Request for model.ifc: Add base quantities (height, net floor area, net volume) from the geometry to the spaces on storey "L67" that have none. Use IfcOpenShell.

First a look at what the model holds.

```python
import ifcopenshell
import ifcopenshell.util.element
import ifcopenshell.util.unit

model = ifcopenshell.open("model.ifc")
print(model.schema)
for unit_type in ("LENGTHUNIT", "AREAUNIT", "VOLUMEUNIT"):
    print(unit_type, ifcopenshell.util.unit.calculate_unit_scale(model, unit_type))
storey = next(s for s in model.by_type("IfcBuildingStorey") if s.Name == "L67")
spaces = [e for e in ifcopenshell.util.element.get_decomposition(storey) if e.is_a("IfcSpace")]
for e in sorted(spaces, key=lambda e: e.id()):
    print(e.id(), e.is_a(), e.Name, list(ifcopenshell.util.element.get_psets(e, qtos_only=True)), sep=" | ")
```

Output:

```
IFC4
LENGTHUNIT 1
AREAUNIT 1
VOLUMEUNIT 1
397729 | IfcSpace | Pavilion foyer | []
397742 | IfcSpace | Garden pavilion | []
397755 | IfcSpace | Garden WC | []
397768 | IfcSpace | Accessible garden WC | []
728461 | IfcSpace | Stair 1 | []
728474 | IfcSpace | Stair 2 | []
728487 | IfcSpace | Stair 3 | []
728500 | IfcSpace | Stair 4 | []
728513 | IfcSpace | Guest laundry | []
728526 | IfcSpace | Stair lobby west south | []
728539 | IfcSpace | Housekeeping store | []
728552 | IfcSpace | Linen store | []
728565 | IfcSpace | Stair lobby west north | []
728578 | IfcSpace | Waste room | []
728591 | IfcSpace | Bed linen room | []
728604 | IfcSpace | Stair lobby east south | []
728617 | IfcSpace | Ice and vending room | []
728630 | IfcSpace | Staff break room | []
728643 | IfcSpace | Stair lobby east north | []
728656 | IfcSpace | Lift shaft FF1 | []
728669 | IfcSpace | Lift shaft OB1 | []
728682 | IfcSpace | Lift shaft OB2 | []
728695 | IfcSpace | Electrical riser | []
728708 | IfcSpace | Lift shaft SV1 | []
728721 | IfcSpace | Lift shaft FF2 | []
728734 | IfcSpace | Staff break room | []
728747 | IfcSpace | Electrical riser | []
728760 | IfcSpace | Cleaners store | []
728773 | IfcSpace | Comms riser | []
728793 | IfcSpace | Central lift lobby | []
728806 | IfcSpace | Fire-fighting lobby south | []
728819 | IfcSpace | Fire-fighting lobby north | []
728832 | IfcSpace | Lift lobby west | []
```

```python
import ifcopenshell
import ifcopenshell.api.pset
import ifcopenshell.geom
import ifcopenshell.util.element
import ifcopenshell.util.shape
import ifcopenshell.util.unit

model = ifcopenshell.open("model.ifc")
unit_scale = ifcopenshell.util.unit.calculate_unit_scale(model)
area_scale = ifcopenshell.util.unit.calculate_unit_scale(model, "AREAUNIT")
volume_scale = ifcopenshell.util.unit.calculate_unit_scale(model, "VOLUMEUNIT")
settings = ifcopenshell.geom.settings()

storey = next(s for s in model.by_type("IfcBuildingStorey") if s.Name == "L67")
spaces = [e for e in ifcopenshell.util.element.get_decomposition(storey) if e.is_a("IfcSpace")]

for e in sorted(spaces, key=lambda e: e.id()):
    if ifcopenshell.util.element.get_psets(e, qtos_only=True, should_inherit=False):
        continue
    # Geometry comes back in metres, in the element's own axes.
    shape = ifcopenshell.geom.create_shape(settings, e)
    values = {
        "Height": ifcopenshell.util.shape.get_z(shape.geometry) / unit_scale,
        "NetFloorArea": ifcopenshell.util.shape.get_footprint_area(shape.geometry) / area_scale,
        "NetVolume": ifcopenshell.util.shape.get_volume(shape.geometry) / volume_scale,
    }
    qto = ifcopenshell.api.pset.add_qto(model, product=e, name="Qto_SpaceBaseQuantities")
    ifcopenshell.api.pset.edit_qto(model, qto=qto, properties=values)
    print(e.id(), {k: round(v, 3) for k, v in values.items()})

model.write("model_edited.ifc")
```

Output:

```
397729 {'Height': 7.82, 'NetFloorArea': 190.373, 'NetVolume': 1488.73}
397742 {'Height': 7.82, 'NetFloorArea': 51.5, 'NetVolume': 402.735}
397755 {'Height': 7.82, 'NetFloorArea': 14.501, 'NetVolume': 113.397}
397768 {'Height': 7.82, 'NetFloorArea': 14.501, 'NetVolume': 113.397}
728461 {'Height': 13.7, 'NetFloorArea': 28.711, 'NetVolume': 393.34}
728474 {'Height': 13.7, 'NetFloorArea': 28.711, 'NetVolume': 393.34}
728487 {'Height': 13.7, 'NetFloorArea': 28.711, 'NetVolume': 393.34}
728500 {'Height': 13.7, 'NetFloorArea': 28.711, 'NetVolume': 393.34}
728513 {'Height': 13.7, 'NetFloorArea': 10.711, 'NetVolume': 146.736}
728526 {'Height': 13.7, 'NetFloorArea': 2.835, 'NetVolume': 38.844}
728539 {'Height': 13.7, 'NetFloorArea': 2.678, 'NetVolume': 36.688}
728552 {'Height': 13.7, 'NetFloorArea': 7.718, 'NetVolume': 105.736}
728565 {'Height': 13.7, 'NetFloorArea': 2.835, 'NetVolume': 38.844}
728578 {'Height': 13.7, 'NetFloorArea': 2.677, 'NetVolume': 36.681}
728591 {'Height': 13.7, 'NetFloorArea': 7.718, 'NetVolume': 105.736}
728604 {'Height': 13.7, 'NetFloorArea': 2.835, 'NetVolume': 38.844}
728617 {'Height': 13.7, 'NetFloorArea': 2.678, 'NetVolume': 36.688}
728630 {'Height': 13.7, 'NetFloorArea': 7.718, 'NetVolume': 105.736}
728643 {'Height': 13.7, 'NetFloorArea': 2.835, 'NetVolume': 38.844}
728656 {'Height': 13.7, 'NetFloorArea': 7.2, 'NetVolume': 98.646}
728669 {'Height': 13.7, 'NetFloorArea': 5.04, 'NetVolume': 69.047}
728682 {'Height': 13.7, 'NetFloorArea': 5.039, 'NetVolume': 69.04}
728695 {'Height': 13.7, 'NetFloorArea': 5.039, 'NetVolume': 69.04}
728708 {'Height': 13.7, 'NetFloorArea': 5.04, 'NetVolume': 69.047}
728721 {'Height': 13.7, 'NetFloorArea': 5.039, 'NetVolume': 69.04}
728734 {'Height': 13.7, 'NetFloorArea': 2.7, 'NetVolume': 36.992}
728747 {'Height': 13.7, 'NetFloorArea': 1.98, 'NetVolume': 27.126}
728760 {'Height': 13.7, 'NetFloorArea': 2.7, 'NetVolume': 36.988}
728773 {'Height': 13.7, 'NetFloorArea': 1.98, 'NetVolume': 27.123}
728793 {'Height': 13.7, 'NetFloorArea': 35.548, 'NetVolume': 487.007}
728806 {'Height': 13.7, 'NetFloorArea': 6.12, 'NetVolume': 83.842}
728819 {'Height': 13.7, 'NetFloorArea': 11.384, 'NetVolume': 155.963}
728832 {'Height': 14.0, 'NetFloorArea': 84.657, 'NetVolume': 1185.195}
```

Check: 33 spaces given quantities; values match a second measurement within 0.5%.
